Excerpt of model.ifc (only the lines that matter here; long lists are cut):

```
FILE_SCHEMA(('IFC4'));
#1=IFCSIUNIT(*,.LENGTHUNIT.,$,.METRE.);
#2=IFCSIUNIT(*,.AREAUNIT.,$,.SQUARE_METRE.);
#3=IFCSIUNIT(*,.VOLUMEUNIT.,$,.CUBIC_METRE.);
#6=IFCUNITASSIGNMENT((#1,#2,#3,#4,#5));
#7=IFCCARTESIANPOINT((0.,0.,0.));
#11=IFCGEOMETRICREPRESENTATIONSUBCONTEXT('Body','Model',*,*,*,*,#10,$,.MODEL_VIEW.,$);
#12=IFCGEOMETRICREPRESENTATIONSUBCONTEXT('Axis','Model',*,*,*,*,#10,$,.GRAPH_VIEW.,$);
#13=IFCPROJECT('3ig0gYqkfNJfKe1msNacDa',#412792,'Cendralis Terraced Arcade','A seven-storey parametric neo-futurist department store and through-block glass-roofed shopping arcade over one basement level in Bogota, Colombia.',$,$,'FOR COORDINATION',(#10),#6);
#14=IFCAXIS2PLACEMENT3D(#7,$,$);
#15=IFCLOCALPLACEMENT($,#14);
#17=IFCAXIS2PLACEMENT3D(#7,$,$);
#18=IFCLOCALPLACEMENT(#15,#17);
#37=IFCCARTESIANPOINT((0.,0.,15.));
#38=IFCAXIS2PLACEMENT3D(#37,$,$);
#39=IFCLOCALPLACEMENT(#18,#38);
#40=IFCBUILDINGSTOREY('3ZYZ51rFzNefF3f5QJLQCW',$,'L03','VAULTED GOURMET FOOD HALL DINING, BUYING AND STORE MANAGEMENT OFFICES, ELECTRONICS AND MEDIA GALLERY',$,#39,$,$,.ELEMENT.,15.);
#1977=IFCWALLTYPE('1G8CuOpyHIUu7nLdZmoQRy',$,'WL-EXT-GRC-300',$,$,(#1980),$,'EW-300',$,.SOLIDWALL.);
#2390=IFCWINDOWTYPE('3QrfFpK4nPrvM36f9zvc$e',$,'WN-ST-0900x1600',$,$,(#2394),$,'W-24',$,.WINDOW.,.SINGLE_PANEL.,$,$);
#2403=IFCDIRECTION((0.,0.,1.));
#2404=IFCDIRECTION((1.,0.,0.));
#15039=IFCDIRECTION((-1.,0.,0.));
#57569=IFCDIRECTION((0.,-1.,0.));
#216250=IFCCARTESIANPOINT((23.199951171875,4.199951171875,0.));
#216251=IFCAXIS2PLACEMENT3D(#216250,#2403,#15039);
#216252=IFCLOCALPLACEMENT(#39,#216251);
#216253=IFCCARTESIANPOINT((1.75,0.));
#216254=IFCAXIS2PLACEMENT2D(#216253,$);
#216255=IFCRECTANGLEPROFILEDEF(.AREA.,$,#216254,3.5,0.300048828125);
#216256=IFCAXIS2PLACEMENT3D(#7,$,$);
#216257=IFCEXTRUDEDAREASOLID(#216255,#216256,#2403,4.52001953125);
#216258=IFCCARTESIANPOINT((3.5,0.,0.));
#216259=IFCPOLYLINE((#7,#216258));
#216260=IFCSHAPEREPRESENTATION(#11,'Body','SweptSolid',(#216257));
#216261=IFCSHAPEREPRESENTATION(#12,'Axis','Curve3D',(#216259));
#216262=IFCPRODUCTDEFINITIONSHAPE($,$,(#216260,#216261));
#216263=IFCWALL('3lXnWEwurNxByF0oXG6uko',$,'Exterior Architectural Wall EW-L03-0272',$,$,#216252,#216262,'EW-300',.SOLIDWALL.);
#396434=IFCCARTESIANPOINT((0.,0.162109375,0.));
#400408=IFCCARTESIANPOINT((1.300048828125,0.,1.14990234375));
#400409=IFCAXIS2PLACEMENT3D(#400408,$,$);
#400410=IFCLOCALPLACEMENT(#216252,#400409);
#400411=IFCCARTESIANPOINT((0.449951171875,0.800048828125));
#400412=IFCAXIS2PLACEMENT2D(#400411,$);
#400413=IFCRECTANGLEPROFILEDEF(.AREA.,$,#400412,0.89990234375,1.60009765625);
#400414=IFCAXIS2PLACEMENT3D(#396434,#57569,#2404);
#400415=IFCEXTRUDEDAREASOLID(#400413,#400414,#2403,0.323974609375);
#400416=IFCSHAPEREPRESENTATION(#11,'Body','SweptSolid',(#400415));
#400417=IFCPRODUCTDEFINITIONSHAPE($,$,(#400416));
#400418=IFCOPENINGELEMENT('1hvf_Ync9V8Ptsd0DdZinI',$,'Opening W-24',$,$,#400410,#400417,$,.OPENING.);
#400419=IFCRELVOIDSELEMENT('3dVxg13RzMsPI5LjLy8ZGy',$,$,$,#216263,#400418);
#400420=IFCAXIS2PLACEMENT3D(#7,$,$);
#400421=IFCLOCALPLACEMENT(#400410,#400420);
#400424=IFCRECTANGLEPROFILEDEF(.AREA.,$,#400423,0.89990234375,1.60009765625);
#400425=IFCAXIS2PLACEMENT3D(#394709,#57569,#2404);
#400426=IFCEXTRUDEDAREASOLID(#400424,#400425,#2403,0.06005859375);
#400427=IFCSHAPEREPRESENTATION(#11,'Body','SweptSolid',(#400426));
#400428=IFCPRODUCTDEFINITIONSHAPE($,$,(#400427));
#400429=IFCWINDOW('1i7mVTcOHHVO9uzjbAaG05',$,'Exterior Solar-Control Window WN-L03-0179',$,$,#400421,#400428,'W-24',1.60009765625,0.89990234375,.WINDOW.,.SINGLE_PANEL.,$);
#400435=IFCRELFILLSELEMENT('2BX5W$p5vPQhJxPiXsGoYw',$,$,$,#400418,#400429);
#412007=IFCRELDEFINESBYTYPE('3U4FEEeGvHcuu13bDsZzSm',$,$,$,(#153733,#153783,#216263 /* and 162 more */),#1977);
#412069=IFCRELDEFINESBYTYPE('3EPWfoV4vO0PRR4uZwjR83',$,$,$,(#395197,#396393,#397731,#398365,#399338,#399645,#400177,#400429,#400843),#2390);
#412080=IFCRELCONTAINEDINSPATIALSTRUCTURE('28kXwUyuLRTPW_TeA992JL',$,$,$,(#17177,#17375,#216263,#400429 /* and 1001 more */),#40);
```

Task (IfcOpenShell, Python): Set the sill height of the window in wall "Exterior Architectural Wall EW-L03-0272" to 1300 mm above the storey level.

```python
import numpy as np
import ifcopenshell
import ifcopenshell.api.geometry
import ifcopenshell.geom
import ifcopenshell.util.element
import ifcopenshell.util.placement
import ifcopenshell.util.shape
import ifcopenshell.util.unit

model = ifcopenshell.open("model.ifc")
unit_scale = ifcopenshell.util.unit.calculate_unit_scale(model)

window = model.by_guid("1i7mVTcOHHVO9uzjbAaG05")
opening = window.FillsVoids[0].RelatingOpeningElement
storey = ifcopenshell.util.element.get_container(window, ifc_class="IfcBuildingStorey")
level = ifcopenshell.util.placement.get_local_placement(storey.ObjectPlacement)[2, 3]

# The opening's origin need not be at the sill, so measure its lowest point.
shape = ifcopenshell.geom.create_shape(ifcopenshell.geom.settings(), opening)
bottom = ifcopenshell.util.shape.get_shape_bottom_elevation(shape, shape.geometry) / unit_scale
dz = level + 1.3 - bottom

shift = np.array([0.0, 0.0, dz])
# The window is placed relative to its opening, so it follows when the opening moves.
matrix = ifcopenshell.util.placement.get_local_placement(opening.ObjectPlacement)
matrix[:3, 3] += shift
ifcopenshell.api.geometry.edit_object_placement(
    model, product=opening, matrix=matrix, is_si=False, should_transform_children=True
)

print(f"moved by {dz * unit_scale:+.3f} m")

model.write("model_rev.ifc")
```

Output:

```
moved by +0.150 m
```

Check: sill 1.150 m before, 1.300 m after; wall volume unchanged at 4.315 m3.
